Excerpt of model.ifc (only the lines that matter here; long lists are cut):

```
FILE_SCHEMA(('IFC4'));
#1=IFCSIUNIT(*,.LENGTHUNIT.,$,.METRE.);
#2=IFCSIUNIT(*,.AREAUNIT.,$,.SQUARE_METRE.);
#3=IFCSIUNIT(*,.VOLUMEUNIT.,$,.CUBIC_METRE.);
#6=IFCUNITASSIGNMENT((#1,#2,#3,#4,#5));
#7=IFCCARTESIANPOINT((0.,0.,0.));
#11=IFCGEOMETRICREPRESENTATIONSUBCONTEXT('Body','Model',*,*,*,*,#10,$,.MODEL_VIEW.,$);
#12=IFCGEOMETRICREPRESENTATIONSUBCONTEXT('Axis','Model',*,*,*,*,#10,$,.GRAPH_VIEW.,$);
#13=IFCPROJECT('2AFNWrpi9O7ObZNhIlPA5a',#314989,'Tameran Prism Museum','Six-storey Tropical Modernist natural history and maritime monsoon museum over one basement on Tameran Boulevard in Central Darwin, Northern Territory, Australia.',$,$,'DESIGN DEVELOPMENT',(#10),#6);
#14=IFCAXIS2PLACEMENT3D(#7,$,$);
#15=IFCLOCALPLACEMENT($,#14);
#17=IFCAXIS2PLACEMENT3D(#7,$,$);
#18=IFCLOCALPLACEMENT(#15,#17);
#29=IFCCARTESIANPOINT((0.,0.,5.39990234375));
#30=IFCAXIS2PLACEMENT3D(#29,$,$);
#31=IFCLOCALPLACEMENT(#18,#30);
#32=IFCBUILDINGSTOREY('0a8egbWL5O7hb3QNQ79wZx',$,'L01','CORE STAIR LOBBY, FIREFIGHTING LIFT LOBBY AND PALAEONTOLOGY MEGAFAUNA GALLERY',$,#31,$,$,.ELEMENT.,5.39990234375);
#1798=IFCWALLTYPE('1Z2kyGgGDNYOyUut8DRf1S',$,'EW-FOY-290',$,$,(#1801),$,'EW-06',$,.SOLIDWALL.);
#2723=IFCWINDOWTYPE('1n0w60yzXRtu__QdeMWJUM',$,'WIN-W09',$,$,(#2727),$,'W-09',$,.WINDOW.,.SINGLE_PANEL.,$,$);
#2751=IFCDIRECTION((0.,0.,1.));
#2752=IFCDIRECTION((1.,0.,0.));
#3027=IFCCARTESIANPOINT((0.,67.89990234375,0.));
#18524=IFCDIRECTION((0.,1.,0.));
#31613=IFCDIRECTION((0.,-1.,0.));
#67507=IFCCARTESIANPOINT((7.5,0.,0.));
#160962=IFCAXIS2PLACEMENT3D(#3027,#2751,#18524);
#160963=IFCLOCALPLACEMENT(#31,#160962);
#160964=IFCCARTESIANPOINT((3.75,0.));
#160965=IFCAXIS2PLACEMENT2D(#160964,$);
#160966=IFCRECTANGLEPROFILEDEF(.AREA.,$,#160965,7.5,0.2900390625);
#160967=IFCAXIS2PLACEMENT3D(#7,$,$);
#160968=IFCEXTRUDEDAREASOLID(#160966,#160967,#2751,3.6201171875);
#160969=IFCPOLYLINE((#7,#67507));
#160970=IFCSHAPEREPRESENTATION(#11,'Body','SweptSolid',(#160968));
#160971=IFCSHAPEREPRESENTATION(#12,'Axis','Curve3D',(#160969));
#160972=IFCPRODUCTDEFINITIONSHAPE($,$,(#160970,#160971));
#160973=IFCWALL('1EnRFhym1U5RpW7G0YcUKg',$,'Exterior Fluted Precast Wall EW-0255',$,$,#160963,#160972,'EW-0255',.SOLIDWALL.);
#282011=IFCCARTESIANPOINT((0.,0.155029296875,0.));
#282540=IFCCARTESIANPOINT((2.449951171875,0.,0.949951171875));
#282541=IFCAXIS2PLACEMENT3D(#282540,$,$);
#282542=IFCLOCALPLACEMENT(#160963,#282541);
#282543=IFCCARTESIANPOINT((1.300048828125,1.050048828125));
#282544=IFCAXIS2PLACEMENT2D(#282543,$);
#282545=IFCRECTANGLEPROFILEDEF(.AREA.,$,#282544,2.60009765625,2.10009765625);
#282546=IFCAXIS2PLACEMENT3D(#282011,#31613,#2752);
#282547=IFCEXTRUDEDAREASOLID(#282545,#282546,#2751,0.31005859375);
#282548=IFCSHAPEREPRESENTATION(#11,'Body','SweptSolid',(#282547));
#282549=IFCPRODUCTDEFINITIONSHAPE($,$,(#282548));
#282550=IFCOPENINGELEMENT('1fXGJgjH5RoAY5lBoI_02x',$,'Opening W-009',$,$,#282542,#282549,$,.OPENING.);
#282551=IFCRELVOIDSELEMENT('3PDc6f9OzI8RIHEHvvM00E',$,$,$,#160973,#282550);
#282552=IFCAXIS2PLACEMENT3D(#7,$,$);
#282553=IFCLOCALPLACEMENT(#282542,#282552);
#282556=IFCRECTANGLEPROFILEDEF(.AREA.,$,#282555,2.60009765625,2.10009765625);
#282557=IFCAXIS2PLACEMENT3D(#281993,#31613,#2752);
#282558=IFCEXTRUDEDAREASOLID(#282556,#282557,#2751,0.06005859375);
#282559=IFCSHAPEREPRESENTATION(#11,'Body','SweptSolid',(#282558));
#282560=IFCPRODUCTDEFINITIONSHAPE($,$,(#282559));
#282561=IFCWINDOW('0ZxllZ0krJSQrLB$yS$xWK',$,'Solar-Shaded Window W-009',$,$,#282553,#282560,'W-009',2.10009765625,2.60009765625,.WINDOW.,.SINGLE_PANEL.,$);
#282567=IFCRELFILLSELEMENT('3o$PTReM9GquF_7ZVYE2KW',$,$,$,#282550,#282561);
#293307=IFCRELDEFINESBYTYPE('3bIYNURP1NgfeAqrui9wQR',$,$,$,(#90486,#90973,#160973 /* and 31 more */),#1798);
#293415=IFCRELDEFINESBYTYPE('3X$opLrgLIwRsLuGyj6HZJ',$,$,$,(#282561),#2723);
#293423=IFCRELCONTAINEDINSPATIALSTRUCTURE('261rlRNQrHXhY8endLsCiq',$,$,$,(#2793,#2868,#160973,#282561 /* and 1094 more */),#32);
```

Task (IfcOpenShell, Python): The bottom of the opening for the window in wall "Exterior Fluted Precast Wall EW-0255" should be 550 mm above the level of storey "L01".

```python
import numpy as np
import ifcopenshell
import ifcopenshell.api.geometry
import ifcopenshell.geom
import ifcopenshell.util.element
import ifcopenshell.util.placement
import ifcopenshell.util.shape
import ifcopenshell.util.unit

model = ifcopenshell.open("model.ifc")
unit_scale = ifcopenshell.util.unit.calculate_unit_scale(model)

window = model.by_guid("0ZxllZ0krJSQrLB$yS$xWK")
opening = window.FillsVoids[0].RelatingOpeningElement
storey = ifcopenshell.util.element.get_container(window, ifc_class="IfcBuildingStorey")
level = ifcopenshell.util.placement.get_local_placement(storey.ObjectPlacement)[2, 3]

# The opening's origin need not be at the sill, so measure its lowest point.
shape = ifcopenshell.geom.create_shape(ifcopenshell.geom.settings(), opening)
bottom = ifcopenshell.util.shape.get_shape_bottom_elevation(shape, shape.geometry) / unit_scale
dz = level + 0.55 / unit_scale - bottom

shift = np.array([0.0, 0.0, dz])
# The window is placed relative to its opening, so it follows when the opening moves.
matrix = ifcopenshell.util.placement.get_local_placement(opening.ObjectPlacement)
matrix[:3, 3] += shift
ifcopenshell.api.geometry.edit_object_placement(
    model, product=opening, matrix=matrix, is_si=False, should_transform_children=True
)

print(f"moved by {dz * unit_scale:+.3f} m")

model.write("model_rev.ifc")
```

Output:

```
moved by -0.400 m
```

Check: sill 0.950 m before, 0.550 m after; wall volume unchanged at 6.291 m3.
